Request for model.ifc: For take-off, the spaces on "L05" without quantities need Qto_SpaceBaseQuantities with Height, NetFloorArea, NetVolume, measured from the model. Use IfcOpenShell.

First a look at what the model holds.

```python
import ifcopenshell
import ifcopenshell.util.element
import ifcopenshell.util.unit

model = ifcopenshell.open("model.ifc")
print(model.schema)
for unit_type in ("LENGTHUNIT", "AREAUNIT", "VOLUMEUNIT"):
    print(unit_type, ifcopenshell.util.unit.calculate_unit_scale(model, unit_type))
storey = next(s for s in model.by_type("IfcBuildingStorey") if s.Name == "L05")
spaces = [e for e in ifcopenshell.util.element.get_decomposition(storey) if e.is_a("IfcSpace")]
for e in sorted(spaces, key=lambda e: e.id()):
    print(e.id(), e.is_a(), e.Name, list(ifcopenshell.util.element.get_psets(e, qtos_only=True)), sep=" | ")
```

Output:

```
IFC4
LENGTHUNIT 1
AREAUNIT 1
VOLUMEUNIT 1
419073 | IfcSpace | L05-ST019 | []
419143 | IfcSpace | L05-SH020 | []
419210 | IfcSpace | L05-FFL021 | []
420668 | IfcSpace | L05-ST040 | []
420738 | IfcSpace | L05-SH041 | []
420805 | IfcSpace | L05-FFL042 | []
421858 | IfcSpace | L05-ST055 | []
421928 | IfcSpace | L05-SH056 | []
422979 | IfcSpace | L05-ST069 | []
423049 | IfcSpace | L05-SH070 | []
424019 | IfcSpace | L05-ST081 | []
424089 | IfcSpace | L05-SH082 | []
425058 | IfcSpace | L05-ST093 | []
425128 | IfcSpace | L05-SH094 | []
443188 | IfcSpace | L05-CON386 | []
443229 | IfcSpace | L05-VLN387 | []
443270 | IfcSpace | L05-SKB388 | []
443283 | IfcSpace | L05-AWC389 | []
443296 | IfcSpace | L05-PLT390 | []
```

```python
import ifcopenshell
import ifcopenshell.api.pset
import ifcopenshell.geom
import ifcopenshell.util.element
import ifcopenshell.util.shape
import ifcopenshell.util.unit

model = ifcopenshell.open("model.ifc")
unit_scale = ifcopenshell.util.unit.calculate_unit_scale(model)
area_scale = ifcopenshell.util.unit.calculate_unit_scale(model, "AREAUNIT")
volume_scale = ifcopenshell.util.unit.calculate_unit_scale(model, "VOLUMEUNIT")
settings = ifcopenshell.geom.settings()

storey = next(s for s in model.by_type("IfcBuildingStorey") if s.Name == "L05")
spaces = [e for e in ifcopenshell.util.element.get_decomposition(storey) if e.is_a("IfcSpace")]

for e in sorted(spaces, key=lambda e: e.id()):
    if ifcopenshell.util.element.get_psets(e, qtos_only=True, should_inherit=False):
        continue
    # Geometry comes back in metres, in the element's own axes.
    shape = ifcopenshell.geom.create_shape(settings, e)
    values = {
        "Height": ifcopenshell.util.shape.get_z(shape.geometry) / unit_scale,
        "NetFloorArea": ifcopenshell.util.shape.get_footprint_area(shape.geometry) / area_scale,
        "NetVolume": ifcopenshell.util.shape.get_volume(shape.geometry) / volume_scale,
    }
    qto = ifcopenshell.api.pset.add_qto(model, product=e, name="Qto_SpaceBaseQuantities")
    ifcopenshell.api.pset.edit_qto(model, qto=qto, properties=values)
    print(e.id(), {k: round(v, 3) for k, v in values.items()})

model.write("model-out.ifc")
```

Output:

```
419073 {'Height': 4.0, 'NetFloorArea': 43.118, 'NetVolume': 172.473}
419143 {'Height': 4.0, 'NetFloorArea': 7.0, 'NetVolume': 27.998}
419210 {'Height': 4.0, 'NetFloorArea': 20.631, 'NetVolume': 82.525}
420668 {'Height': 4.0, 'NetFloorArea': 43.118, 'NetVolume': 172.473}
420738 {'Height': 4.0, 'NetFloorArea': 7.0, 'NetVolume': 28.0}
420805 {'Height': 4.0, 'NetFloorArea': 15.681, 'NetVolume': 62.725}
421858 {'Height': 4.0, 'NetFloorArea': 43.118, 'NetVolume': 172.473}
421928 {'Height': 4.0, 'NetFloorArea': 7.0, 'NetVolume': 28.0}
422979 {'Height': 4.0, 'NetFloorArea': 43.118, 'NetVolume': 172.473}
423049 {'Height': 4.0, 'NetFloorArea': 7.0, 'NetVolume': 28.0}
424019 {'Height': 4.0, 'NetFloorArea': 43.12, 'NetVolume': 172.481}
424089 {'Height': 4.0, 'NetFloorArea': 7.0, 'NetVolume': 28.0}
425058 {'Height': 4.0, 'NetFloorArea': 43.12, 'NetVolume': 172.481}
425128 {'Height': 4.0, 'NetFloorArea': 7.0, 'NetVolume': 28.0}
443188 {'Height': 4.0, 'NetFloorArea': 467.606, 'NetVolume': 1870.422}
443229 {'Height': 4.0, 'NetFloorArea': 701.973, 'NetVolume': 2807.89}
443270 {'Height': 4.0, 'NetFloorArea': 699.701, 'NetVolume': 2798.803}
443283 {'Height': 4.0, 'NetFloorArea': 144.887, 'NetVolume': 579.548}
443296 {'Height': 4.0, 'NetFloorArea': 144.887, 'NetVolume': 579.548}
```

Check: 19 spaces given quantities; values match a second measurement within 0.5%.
